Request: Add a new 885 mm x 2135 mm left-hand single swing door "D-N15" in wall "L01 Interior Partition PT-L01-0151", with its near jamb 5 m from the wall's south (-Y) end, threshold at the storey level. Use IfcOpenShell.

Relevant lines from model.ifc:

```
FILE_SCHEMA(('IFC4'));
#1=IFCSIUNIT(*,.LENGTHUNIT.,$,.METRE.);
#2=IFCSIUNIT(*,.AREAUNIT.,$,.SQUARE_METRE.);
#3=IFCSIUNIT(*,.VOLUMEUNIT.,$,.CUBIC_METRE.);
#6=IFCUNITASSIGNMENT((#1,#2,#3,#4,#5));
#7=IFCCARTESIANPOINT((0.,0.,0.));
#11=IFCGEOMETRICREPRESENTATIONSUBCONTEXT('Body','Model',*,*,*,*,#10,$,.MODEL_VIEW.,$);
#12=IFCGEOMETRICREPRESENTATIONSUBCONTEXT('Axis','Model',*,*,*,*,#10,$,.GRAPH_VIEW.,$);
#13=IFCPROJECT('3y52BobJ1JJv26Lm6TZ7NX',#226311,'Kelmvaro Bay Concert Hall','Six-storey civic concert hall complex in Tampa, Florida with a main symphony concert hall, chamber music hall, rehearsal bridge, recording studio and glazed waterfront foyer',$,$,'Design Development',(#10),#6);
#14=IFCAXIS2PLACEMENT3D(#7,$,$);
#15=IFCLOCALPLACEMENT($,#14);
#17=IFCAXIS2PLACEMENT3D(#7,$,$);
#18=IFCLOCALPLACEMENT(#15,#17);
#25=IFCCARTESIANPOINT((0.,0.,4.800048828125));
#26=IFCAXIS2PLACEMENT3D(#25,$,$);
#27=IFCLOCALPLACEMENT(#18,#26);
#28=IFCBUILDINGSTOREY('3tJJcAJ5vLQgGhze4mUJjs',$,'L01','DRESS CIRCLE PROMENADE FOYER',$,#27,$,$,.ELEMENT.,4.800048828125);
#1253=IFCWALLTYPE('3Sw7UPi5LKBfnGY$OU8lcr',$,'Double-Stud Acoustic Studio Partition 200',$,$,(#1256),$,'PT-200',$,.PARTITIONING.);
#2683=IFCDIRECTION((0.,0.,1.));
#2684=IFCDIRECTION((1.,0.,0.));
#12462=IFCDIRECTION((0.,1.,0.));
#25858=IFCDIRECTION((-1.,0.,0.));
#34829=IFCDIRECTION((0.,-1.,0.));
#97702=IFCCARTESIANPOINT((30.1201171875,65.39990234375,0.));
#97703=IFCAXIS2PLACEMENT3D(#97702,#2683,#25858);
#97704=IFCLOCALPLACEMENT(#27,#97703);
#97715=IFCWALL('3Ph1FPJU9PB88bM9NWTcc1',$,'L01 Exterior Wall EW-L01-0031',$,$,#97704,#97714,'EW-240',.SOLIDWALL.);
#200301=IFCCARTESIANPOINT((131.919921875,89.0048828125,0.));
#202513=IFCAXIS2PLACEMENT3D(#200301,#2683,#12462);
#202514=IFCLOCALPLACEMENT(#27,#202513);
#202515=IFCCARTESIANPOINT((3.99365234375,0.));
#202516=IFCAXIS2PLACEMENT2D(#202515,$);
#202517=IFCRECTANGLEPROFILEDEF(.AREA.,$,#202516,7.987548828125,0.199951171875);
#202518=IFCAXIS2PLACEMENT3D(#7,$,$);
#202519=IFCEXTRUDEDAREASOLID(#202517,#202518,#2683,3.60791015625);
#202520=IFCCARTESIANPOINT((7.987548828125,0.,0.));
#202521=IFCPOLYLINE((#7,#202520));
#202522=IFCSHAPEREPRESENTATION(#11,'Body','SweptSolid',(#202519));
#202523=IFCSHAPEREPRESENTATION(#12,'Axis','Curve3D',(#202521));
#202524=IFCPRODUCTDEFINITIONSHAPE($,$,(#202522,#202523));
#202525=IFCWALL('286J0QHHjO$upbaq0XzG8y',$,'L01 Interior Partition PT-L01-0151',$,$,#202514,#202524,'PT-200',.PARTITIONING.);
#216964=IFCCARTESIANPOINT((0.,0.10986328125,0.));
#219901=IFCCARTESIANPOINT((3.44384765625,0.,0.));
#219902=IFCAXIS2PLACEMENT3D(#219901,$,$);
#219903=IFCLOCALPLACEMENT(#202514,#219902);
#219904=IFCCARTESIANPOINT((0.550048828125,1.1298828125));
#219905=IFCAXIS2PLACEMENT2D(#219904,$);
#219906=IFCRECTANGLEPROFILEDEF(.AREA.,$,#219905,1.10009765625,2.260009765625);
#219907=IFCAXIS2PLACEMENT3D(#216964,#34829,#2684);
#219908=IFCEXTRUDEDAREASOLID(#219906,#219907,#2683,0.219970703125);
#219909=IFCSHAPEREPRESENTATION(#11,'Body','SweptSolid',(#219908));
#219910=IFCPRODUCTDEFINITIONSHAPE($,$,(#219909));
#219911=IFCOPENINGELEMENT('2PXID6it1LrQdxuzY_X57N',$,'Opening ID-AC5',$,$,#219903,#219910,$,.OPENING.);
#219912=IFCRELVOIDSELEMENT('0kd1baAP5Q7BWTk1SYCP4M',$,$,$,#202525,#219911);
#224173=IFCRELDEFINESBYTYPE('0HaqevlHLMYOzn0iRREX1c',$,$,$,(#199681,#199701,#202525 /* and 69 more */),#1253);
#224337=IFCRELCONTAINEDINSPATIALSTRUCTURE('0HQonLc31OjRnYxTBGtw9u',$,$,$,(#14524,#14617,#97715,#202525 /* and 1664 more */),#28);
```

```python
import numpy as np
import ifcopenshell
import ifcopenshell.api.feature
import ifcopenshell.api.geometry
import ifcopenshell.api.root
import ifcopenshell.api.spatial
import ifcopenshell.geom
import ifcopenshell.util.element
import ifcopenshell.util.placement
import ifcopenshell.util.representation
import ifcopenshell.util.shape
import ifcopenshell.util.unit

model = ifcopenshell.open("model.ifc")
unit_scale = ifcopenshell.util.unit.calculate_unit_scale(model)
settings = ifcopenshell.geom.settings()


def volume(element):
    """Net volume in cubic metres, openings subtracted."""
    shape = ifcopenshell.geom.create_shape(settings, element)
    return ifcopenshell.util.shape.get_volume(shape.geometry)


wall = model.by_guid("286J0QHHjO$upbaq0XzG8y")
storey = ifcopenshell.util.element.get_container(wall, ifc_class="IfcBuildingStorey")
context = ifcopenshell.util.representation.get_context(model, "Model", "Body", "MODEL_VIEW")
before = volume(wall)

width, height, from_end, sill = 0.885, 2.135, 5, 0.0  # metres

# The wall runs along its own X axis, and the end named is its -X end.
wall_shape = ifcopenshell.geom.create_shape(settings, wall)
x, y, z = ifcopenshell.util.shape.get_vertices(wall_shape.geometry).T
start = x.min() + from_end
face, thickness = float(y.min()), float(y.max() - y.min())
wall_matrix = ifcopenshell.util.placement.get_local_placement(wall.ObjectPlacement)
level = ifcopenshell.util.placement.get_local_placement(storey.ObjectPlacement)[2, 3]


def in_wall(x, y):
    """Placement at x, y metres in the wall's axes, at sill height."""
    matrix = wall_matrix.copy()
    matrix[:, 3] = wall_matrix @ np.array([x / unit_scale, y / unit_scale, 0.0, 1.0])
    matrix[2, 3] = level + sill / unit_scale
    return matrix


# Opening: a box that overshoots both wall faces by 50 mm.
opening = ifcopenshell.api.root.create_entity(model, ifc_class="IfcOpeningElement", predefined_type="OPENING")
box = ifcopenshell.api.geometry.add_wall_representation(
    model, context=context, length=width, height=height, thickness=thickness + 0.1
)
ifcopenshell.api.geometry.assign_representation(model, product=opening, representation=box)
ifcopenshell.api.geometry.edit_object_placement(model, product=opening, matrix=in_wall(start, face - 0.05), is_si=False)
ifcopenshell.api.feature.add_feature(model, feature=opening, element=wall)

door = ifcopenshell.api.root.create_entity(model, ifc_class="IfcDoor", name="D-N15", predefined_type="DOOR")
door.OverallWidth, door.OverallHeight = width / unit_scale, height / unit_scale
door.OperationType = "SINGLE_SWING_LEFT"
body = ifcopenshell.api.geometry.add_door_representation(
    model,
    context=context,
    overall_width=door.OverallWidth,
    overall_height=door.OverallHeight,
    operation_type="SINGLE_SWING_LEFT",
    lining_properties={"LiningDepth": thickness / unit_scale, "ThresholdDepth": thickness / unit_scale},
)
ifcopenshell.api.geometry.assign_representation(model, product=door, representation=body)
ifcopenshell.api.spatial.assign_container(model, products=[door], relating_structure=storey)
ifcopenshell.api.feature.add_filling(model, opening=opening, element=door)

# The lining spans the wall, so the door starts at the wall face.
ifcopenshell.api.geometry.edit_object_placement(model, product=door, matrix=in_wall(start, face), is_si=False)

after = volume(wall)

print(f"wall volume {before:.3f} -> {after:.3f} m3")

model.write("model_rev.ifc")
```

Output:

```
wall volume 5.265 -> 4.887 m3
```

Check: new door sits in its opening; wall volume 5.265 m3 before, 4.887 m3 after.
